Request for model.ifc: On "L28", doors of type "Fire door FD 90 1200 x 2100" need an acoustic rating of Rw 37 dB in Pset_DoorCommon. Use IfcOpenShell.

First a look at what the model holds.

```python
import ifcopenshell
import ifcopenshell.util.element

model = ifcopenshell.open("model.ifc")
print(model.schema)
storey = next(s for s in model.by_type("IfcBuildingStorey") if s.Name == "L28")
doors = [e for e in ifcopenshell.util.element.get_decomposition(storey) if e.is_a("IfcDoor")]
seen = {}
for e in doors:
    element_type = ifcopenshell.util.element.get_type(e)
    key = (element_type.Name if element_type != e and element_type else None, ifcopenshell.util.element.get_pset(e, "Pset_DoorCommon", "AcousticRating"))
    seen[key] = seen.get(key, 0) + 1
for (name, value), count in sorted(seen.items(), key=str):
    print(count, "x", name, "|", value)
```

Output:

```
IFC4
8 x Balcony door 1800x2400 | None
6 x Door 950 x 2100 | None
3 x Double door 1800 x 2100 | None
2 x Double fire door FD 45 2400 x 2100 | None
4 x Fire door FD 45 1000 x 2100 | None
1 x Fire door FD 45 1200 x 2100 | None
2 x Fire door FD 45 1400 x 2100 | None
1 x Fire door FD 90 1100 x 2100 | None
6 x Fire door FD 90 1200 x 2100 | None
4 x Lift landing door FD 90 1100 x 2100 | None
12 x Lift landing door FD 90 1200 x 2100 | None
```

```python
import ifcopenshell
import ifcopenshell.api.pset
import ifcopenshell.util.element

model = ifcopenshell.open("model.ifc")

storey = next(s for s in model.by_type("IfcBuildingStorey") if s.Name == "L28")
doors = [e for e in ifcopenshell.util.element.get_decomposition(storey) if e.is_a("IfcDoor")]

count = 0
for e in doors:
    element_type = ifcopenshell.util.element.get_type(e)
    if element_type in (None, e) or element_type.Name != "Fire door FD 90 1200 x 2100":
        continue
    found = ifcopenshell.util.element.get_pset(e, "Pset_DoorCommon", should_inherit=False)
    if found:
        pset = model.by_id(found["id"])
        if len(ifcopenshell.util.element.get_elements_by_pset(pset)) > 1:
            pset = ifcopenshell.api.pset.unshare_pset(model, products=[e], pset=pset)[0]
    else:
        pset = ifcopenshell.api.pset.add_pset(model, product=e, name="Pset_DoorCommon")
    ifcopenshell.api.pset.edit_pset(model, pset=pset, properties={"AcousticRating": "Rw 37 dB"})
    count += 1

print(count, "doors updated")

model.write("model_v2.ifc")
```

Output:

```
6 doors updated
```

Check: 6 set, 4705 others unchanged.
